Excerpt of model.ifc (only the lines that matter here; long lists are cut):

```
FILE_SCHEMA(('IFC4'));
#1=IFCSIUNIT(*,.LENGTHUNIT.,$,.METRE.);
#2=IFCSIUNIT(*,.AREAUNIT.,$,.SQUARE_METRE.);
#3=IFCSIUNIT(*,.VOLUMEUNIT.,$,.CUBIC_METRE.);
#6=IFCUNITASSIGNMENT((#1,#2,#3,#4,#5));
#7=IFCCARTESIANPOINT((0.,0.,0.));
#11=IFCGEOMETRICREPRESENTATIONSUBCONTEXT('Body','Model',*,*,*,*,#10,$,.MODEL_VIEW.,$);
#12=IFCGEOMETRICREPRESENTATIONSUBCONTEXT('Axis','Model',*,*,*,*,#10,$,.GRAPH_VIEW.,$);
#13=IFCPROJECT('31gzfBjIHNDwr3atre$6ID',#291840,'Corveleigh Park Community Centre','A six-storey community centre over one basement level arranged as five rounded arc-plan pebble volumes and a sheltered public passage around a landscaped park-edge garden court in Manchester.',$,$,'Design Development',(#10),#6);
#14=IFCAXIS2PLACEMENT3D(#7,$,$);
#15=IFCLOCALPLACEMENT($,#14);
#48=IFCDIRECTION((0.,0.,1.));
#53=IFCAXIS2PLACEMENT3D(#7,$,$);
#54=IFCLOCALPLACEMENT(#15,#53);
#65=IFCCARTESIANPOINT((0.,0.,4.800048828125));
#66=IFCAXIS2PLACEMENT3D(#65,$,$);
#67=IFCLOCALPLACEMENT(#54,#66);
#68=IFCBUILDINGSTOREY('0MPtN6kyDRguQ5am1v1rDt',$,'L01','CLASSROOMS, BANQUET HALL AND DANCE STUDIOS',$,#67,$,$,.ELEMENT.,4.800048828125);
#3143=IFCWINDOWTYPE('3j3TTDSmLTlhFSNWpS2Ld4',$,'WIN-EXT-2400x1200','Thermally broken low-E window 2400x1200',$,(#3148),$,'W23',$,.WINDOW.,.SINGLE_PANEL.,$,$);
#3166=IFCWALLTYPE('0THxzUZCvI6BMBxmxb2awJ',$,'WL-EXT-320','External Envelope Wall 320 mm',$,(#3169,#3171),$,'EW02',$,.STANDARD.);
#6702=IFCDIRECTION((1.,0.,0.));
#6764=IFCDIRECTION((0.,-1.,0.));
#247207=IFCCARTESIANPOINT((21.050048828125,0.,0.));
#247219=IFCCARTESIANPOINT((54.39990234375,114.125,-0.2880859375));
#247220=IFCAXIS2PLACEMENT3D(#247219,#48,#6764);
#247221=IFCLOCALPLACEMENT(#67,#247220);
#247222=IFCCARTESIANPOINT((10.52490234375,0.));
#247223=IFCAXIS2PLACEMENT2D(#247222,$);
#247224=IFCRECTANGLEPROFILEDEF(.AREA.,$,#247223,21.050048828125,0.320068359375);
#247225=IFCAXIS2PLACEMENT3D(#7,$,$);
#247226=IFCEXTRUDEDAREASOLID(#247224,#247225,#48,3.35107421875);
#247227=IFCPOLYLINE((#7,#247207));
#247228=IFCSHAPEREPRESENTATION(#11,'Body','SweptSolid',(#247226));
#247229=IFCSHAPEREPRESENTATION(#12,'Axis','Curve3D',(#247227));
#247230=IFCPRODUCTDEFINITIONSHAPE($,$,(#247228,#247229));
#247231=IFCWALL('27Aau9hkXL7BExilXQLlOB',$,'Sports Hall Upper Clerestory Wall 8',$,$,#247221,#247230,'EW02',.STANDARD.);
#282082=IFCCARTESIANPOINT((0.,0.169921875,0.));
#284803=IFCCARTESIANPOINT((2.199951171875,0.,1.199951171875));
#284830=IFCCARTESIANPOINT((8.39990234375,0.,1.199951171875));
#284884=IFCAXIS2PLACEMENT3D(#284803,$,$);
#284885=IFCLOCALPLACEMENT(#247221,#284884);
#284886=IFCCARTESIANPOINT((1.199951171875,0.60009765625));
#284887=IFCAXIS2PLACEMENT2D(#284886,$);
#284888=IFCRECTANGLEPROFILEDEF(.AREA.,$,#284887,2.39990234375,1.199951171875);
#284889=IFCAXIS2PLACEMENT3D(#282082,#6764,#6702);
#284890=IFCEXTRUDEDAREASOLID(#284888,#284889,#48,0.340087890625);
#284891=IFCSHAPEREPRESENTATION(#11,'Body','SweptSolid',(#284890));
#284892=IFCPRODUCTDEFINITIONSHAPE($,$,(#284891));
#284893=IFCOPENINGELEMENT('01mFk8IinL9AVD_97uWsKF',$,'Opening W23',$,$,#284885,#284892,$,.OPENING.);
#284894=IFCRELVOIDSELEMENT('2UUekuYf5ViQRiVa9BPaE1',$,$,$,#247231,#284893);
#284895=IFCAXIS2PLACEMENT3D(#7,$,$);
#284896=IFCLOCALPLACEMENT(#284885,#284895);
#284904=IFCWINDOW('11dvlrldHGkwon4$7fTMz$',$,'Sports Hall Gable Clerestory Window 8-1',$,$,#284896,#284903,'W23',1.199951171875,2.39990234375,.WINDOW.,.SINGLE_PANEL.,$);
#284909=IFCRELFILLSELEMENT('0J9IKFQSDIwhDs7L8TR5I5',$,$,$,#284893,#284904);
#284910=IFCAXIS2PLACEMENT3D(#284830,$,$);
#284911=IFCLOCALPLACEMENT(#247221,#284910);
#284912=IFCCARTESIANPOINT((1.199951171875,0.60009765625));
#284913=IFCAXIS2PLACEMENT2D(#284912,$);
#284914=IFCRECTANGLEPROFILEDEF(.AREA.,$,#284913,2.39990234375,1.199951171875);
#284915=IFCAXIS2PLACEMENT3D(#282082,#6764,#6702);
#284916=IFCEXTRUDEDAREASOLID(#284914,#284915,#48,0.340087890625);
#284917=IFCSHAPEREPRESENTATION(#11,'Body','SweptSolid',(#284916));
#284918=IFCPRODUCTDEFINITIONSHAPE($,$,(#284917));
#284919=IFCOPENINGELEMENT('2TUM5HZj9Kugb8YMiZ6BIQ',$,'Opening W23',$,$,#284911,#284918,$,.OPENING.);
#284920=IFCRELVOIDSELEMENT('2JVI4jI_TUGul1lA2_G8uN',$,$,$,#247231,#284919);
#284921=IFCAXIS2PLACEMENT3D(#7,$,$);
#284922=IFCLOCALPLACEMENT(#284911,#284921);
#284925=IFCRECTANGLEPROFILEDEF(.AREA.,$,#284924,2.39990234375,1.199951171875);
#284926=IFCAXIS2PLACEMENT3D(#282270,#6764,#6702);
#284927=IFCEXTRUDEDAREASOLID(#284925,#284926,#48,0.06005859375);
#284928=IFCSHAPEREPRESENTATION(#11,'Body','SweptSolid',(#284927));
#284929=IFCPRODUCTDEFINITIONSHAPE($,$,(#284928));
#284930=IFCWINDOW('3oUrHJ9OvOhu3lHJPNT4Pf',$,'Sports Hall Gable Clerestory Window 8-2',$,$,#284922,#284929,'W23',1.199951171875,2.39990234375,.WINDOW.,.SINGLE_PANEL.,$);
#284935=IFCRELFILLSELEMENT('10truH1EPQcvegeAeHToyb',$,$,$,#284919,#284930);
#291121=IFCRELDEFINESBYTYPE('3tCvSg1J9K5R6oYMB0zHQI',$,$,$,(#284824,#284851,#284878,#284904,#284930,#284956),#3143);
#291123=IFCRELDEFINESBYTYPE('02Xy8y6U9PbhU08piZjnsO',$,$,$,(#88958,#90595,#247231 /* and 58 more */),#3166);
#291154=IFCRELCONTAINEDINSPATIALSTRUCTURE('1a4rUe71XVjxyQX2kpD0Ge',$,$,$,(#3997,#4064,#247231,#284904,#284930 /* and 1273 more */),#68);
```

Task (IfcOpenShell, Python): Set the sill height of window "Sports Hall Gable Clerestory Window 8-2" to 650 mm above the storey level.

```python
import numpy as np
import ifcopenshell
import ifcopenshell.api.geometry
import ifcopenshell.geom
import ifcopenshell.util.element
import ifcopenshell.util.placement
import ifcopenshell.util.shape
import ifcopenshell.util.unit

model = ifcopenshell.open("model.ifc")
unit_scale = ifcopenshell.util.unit.calculate_unit_scale(model)

window = model.by_guid("3oUrHJ9OvOhu3lHJPNT4Pf")
opening = window.FillsVoids[0].RelatingOpeningElement
storey = ifcopenshell.util.element.get_container(window, ifc_class="IfcBuildingStorey")
level = ifcopenshell.util.placement.get_local_placement(storey.ObjectPlacement)[2, 3]

# The opening's origin need not be at the sill, so measure its lowest point.
shape = ifcopenshell.geom.create_shape(ifcopenshell.geom.settings(), opening)
bottom = ifcopenshell.util.shape.get_shape_bottom_elevation(shape, shape.geometry) / unit_scale
dz = level + 0.65 - bottom

shift = np.array([0.0, 0.0, dz])
# The window is placed relative to its opening, so it follows when the opening moves.
matrix = ifcopenshell.util.placement.get_local_placement(opening.ObjectPlacement)
matrix[:3, 3] += shift
ifcopenshell.api.geometry.edit_object_placement(
    model, product=opening, matrix=matrix, is_si=False, should_transform_children=True
)

print(f"moved by {dz * unit_scale:+.3f} m")

model.write("model_v2.ifc")
```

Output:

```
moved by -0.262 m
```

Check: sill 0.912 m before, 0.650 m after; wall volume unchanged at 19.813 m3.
